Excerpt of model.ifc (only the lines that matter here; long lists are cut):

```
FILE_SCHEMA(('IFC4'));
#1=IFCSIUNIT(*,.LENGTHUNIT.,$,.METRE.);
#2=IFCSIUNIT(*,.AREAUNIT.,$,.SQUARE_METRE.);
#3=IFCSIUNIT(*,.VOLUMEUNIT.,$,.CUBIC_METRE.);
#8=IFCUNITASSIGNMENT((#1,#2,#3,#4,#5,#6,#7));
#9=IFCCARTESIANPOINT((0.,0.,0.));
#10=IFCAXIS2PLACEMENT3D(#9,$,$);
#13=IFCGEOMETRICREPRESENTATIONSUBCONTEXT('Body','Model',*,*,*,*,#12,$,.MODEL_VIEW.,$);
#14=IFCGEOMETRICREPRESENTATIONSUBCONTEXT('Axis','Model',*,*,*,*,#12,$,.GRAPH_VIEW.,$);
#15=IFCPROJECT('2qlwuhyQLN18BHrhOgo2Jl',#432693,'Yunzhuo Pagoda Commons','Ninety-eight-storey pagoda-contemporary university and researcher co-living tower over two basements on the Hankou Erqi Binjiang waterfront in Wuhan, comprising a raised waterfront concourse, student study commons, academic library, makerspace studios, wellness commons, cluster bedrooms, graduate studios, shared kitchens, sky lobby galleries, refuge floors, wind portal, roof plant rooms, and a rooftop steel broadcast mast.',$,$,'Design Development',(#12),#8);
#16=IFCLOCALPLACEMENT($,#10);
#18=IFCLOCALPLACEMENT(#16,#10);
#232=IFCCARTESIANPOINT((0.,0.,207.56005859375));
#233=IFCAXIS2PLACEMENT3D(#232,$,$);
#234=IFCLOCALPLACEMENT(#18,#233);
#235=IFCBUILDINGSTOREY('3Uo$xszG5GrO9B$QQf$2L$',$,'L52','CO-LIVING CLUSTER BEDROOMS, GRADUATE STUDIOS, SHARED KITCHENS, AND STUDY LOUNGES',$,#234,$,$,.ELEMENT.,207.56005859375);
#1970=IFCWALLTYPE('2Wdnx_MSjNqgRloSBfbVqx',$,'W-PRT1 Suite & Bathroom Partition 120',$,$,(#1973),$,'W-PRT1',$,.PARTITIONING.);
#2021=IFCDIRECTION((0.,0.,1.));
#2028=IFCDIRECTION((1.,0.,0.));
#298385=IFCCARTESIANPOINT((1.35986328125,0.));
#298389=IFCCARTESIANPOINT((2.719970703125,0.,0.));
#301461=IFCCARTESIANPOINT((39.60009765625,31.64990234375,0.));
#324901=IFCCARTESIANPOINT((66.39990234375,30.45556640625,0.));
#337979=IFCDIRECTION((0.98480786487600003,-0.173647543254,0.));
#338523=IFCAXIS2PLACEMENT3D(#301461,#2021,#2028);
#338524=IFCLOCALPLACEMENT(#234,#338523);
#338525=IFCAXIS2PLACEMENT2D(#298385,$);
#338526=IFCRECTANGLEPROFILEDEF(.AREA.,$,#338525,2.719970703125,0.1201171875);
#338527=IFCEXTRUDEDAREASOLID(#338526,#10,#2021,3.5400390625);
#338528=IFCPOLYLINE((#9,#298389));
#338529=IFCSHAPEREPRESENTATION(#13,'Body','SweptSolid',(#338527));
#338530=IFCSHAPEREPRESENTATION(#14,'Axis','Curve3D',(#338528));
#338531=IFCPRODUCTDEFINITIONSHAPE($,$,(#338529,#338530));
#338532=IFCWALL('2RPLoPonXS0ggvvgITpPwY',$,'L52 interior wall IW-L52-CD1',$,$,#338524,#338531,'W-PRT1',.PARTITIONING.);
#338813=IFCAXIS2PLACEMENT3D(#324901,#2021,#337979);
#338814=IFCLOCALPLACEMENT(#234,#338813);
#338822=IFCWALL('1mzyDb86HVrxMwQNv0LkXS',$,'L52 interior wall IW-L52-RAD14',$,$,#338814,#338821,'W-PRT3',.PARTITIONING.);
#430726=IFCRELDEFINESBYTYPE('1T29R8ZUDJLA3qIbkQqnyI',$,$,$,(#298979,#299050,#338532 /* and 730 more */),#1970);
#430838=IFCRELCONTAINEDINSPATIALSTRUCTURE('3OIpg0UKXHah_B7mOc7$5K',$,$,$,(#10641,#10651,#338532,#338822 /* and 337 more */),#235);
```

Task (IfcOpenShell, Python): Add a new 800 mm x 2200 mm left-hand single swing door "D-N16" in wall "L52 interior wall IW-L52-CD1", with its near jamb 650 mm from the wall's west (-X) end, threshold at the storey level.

```python
import numpy as np
import ifcopenshell
import ifcopenshell.api.feature
import ifcopenshell.api.geometry
import ifcopenshell.api.root
import ifcopenshell.api.spatial
import ifcopenshell.geom
import ifcopenshell.util.element
import ifcopenshell.util.placement
import ifcopenshell.util.representation
import ifcopenshell.util.shape
import ifcopenshell.util.unit

model = ifcopenshell.open("model.ifc")
unit_scale = ifcopenshell.util.unit.calculate_unit_scale(model)
settings = ifcopenshell.geom.settings()


def volume(element):
    """Net volume in cubic metres, openings subtracted."""
    shape = ifcopenshell.geom.create_shape(settings, element)
    return ifcopenshell.util.shape.get_volume(shape.geometry)


wall = model.by_guid("2RPLoPonXS0ggvvgITpPwY")
storey = ifcopenshell.util.element.get_container(wall, ifc_class="IfcBuildingStorey")
context = ifcopenshell.util.representation.get_context(model, "Model", "Body", "MODEL_VIEW")
before = volume(wall)

width, height, from_end, sill = 0.8, 2.2, 0.65, 0.0  # metres

# The wall runs along its own X axis, and the end named is its -X end.
wall_shape = ifcopenshell.geom.create_shape(settings, wall)
x, y, z = ifcopenshell.util.shape.get_vertices(wall_shape.geometry).T
start = x.min() + from_end
face, thickness = float(y.min()), float(y.max() - y.min())
wall_matrix = ifcopenshell.util.placement.get_local_placement(wall.ObjectPlacement)
level = ifcopenshell.util.placement.get_local_placement(storey.ObjectPlacement)[2, 3]


def in_wall(x, y):
    """Placement at x, y metres in the wall's axes, at sill height."""
    matrix = wall_matrix.copy()
    matrix[:, 3] = wall_matrix @ np.array([x / unit_scale, y / unit_scale, 0.0, 1.0])
    matrix[2, 3] = level + sill / unit_scale
    return matrix


# Opening: a box that overshoots both wall faces by 50 mm.
opening = ifcopenshell.api.root.create_entity(model, ifc_class="IfcOpeningElement", predefined_type="OPENING")
box = ifcopenshell.api.geometry.add_wall_representation(
    model, context=context, length=width, height=height, thickness=thickness + 0.1
)
ifcopenshell.api.geometry.assign_representation(model, product=opening, representation=box)
ifcopenshell.api.geometry.edit_object_placement(model, product=opening, matrix=in_wall(start, face - 0.05), is_si=False)
ifcopenshell.api.feature.add_feature(model, feature=opening, element=wall)

door = ifcopenshell.api.root.create_entity(model, ifc_class="IfcDoor", name="D-N16", predefined_type="DOOR")
door.OverallWidth, door.OverallHeight = width / unit_scale, height / unit_scale
door.OperationType = "SINGLE_SWING_LEFT"
body = ifcopenshell.api.geometry.add_door_representation(
    model,
    context=context,
    overall_width=door.OverallWidth,
    overall_height=door.OverallHeight,
    operation_type="SINGLE_SWING_LEFT",
    lining_properties={"LiningDepth": thickness / unit_scale, "ThresholdDepth": thickness / unit_scale},
)
ifcopenshell.api.geometry.assign_representation(model, product=door, representation=body)
ifcopenshell.api.spatial.assign_container(model, products=[door], relating_structure=storey)
ifcopenshell.api.feature.add_filling(model, opening=opening, element=door)

# The lining spans the wall, so the door starts at the wall face.
ifcopenshell.api.geometry.edit_object_placement(model, product=door, matrix=in_wall(start, face), is_si=False)

after = volume(wall)

print(f"wall volume {before:.3f} -> {after:.3f} m3")

model.write("model_edited.ifc")
```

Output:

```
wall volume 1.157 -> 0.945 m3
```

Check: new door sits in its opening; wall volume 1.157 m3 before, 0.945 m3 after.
